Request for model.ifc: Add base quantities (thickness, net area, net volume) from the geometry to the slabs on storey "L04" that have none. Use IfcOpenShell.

First a look at what the model holds.

```python
import ifcopenshell
import ifcopenshell.util.element
import ifcopenshell.util.unit

model = ifcopenshell.open("model.ifc")
print(model.schema)
for unit_type in ("LENGTHUNIT", "AREAUNIT", "VOLUMEUNIT"):
    print(unit_type, ifcopenshell.util.unit.calculate_unit_scale(model, unit_type))
storey = next(s for s in model.by_type("IfcBuildingStorey") if s.Name == "L04")
slabs = [e for e in ifcopenshell.util.element.get_decomposition(storey) if e.is_a("IfcSlab")]
for e in sorted(slabs, key=lambda e: e.id()):
    print(e.id(), e.is_a(), e.Name, list(ifcopenshell.util.element.get_psets(e, qtos_only=True)), sep=" | ")
```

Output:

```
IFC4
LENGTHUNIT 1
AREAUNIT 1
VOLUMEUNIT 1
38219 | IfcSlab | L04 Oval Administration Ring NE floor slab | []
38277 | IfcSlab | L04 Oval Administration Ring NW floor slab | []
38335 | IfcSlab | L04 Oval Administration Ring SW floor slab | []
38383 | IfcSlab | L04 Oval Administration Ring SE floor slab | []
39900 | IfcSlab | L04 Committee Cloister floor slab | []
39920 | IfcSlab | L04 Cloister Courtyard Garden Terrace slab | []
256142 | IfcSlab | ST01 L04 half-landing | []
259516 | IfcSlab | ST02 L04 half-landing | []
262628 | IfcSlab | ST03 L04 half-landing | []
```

```python
import ifcopenshell
import ifcopenshell.api.pset
import ifcopenshell.geom
import ifcopenshell.util.element
import ifcopenshell.util.shape
import ifcopenshell.util.unit

model = ifcopenshell.open("model.ifc")
unit_scale = ifcopenshell.util.unit.calculate_unit_scale(model)
area_scale = ifcopenshell.util.unit.calculate_unit_scale(model, "AREAUNIT")
volume_scale = ifcopenshell.util.unit.calculate_unit_scale(model, "VOLUMEUNIT")
settings = ifcopenshell.geom.settings()

storey = next(s for s in model.by_type("IfcBuildingStorey") if s.Name == "L04")
slabs = [e for e in ifcopenshell.util.element.get_decomposition(storey) if e.is_a("IfcSlab")]

for e in sorted(slabs, key=lambda e: e.id()):
    if ifcopenshell.util.element.get_psets(e, qtos_only=True, should_inherit=False):
        continue
    # Geometry comes back in metres, in the element's own axes.
    shape = ifcopenshell.geom.create_shape(settings, e)
    values = {
        "Width": ifcopenshell.util.shape.get_z(shape.geometry) / unit_scale,
        "NetArea": ifcopenshell.util.shape.get_footprint_area(shape.geometry) / area_scale,
        "NetVolume": ifcopenshell.util.shape.get_volume(shape.geometry) / volume_scale,
    }
    qto = ifcopenshell.api.pset.add_qto(model, product=e, name="Qto_SlabBaseQuantities")
    ifcopenshell.api.pset.edit_qto(model, qto=qto, properties=values)
    print(e.id(), {k: round(v, 3) for k, v in values.items()})

model.write("model_updated.ifc")
```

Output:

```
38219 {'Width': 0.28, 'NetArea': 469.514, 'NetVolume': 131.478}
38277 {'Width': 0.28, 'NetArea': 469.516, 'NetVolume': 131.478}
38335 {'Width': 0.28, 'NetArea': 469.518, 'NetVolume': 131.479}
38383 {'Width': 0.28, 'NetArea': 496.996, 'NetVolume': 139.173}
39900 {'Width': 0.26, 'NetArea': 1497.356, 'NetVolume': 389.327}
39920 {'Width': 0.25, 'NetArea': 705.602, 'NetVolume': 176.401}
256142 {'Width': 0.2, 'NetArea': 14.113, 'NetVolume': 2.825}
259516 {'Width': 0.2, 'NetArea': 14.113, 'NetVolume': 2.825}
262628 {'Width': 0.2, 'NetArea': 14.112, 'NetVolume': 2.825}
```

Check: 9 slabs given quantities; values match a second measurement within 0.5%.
